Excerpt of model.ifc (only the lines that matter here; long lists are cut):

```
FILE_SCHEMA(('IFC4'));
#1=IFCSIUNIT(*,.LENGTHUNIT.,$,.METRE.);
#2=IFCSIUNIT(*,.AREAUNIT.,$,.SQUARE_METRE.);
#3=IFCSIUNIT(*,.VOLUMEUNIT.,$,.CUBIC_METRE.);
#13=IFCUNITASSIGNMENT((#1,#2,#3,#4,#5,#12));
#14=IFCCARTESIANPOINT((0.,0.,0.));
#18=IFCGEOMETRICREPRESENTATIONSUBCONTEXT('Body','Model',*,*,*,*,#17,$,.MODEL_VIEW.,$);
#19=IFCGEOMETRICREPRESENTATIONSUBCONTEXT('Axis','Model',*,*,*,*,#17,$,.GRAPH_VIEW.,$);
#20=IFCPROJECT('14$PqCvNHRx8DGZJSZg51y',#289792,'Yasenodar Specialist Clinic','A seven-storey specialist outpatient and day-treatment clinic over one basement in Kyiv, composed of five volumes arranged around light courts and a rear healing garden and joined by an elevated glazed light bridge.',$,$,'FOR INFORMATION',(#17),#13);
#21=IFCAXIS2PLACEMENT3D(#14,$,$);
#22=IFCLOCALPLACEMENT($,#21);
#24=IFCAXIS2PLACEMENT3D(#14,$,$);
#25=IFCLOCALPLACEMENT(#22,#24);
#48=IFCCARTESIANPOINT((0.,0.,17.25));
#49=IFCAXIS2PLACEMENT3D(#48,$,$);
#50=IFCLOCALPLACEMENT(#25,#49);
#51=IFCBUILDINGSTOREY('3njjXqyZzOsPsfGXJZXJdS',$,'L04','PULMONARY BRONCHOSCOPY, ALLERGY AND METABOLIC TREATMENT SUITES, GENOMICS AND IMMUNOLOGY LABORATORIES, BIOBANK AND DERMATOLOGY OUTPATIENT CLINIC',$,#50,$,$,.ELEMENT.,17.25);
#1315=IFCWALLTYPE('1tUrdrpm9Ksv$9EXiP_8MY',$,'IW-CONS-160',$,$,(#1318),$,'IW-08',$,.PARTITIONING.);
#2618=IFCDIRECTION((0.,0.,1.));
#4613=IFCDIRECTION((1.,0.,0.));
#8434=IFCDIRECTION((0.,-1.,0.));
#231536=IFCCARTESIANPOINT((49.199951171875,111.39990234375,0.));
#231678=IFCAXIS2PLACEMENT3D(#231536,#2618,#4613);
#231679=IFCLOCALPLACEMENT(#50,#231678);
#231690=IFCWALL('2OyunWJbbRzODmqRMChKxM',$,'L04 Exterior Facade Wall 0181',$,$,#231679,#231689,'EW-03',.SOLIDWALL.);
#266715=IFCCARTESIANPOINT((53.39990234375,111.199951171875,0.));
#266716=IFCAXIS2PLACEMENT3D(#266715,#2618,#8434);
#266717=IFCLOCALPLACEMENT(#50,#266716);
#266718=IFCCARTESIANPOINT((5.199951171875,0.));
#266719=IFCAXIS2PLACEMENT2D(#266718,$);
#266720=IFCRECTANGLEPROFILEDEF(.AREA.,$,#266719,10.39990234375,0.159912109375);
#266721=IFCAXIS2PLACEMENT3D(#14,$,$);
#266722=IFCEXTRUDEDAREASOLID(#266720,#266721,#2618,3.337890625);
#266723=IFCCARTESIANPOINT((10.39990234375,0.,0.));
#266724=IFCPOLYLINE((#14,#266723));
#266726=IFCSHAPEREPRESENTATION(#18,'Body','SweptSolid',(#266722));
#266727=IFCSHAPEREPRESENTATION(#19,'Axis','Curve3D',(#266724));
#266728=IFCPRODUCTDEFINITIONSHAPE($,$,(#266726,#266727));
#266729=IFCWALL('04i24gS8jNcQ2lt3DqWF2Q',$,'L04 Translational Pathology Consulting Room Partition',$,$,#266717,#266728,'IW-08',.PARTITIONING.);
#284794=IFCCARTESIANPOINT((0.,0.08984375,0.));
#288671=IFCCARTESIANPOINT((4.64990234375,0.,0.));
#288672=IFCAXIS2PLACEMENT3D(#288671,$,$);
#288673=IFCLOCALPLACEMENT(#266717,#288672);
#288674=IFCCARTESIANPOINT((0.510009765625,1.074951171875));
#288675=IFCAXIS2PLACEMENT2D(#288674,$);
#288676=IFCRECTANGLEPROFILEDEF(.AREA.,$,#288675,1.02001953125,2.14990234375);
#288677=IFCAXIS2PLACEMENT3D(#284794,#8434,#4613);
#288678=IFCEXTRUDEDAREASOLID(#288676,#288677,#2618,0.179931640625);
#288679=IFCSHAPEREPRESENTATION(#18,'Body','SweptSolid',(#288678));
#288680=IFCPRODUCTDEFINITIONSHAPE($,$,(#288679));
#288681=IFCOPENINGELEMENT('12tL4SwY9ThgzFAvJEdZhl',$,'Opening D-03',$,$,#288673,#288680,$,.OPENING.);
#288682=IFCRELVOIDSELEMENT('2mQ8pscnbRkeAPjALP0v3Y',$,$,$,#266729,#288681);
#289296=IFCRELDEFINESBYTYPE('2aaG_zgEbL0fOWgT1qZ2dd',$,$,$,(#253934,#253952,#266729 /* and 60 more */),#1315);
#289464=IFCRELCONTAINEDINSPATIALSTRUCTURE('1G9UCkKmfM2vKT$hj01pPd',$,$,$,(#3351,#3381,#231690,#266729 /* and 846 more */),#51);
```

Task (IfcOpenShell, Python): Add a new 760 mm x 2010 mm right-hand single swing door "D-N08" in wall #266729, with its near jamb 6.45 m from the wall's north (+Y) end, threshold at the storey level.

```python
import numpy as np
import ifcopenshell
import ifcopenshell.api.feature
import ifcopenshell.api.geometry
import ifcopenshell.api.root
import ifcopenshell.api.spatial
import ifcopenshell.geom
import ifcopenshell.util.element
import ifcopenshell.util.placement
import ifcopenshell.util.representation
import ifcopenshell.util.shape
import ifcopenshell.util.unit

model = ifcopenshell.open("model.ifc")
unit_scale = ifcopenshell.util.unit.calculate_unit_scale(model)
settings = ifcopenshell.geom.settings()


def volume(element):
    """Net volume in cubic metres, openings subtracted."""
    shape = ifcopenshell.geom.create_shape(settings, element)
    return ifcopenshell.util.shape.get_volume(shape.geometry)


wall = model.by_id(266729)
storey = ifcopenshell.util.element.get_container(wall, ifc_class="IfcBuildingStorey")
context = ifcopenshell.util.representation.get_context(model, "Model", "Body", "MODEL_VIEW")
before = volume(wall)

width, height, from_end, sill = 0.76, 2.01, 6.45, 0.0  # metres

# The wall runs along its own X axis, and the end named is its -X end.
wall_shape = ifcopenshell.geom.create_shape(settings, wall)
x, y, z = ifcopenshell.util.shape.get_vertices(wall_shape.geometry).T
start = x.min() + from_end
face, thickness = float(y.min()), float(y.max() - y.min())
wall_matrix = ifcopenshell.util.placement.get_local_placement(wall.ObjectPlacement)
level = ifcopenshell.util.placement.get_local_placement(storey.ObjectPlacement)[2, 3]


def in_wall(x, y):
    """Placement at x, y metres in the wall's axes, at sill height."""
    matrix = wall_matrix.copy()
    matrix[:, 3] = wall_matrix @ np.array([x / unit_scale, y / unit_scale, 0.0, 1.0])
    matrix[2, 3] = level + sill / unit_scale
    return matrix


# Opening: a box that overshoots both wall faces by 50 mm.
opening = ifcopenshell.api.root.create_entity(model, ifc_class="IfcOpeningElement", predefined_type="OPENING")
box = ifcopenshell.api.geometry.add_wall_representation(
    model, context=context, length=width, height=height, thickness=thickness + 0.1
)
ifcopenshell.api.geometry.assign_representation(model, product=opening, representation=box)
ifcopenshell.api.geometry.edit_object_placement(model, product=opening, matrix=in_wall(start, face - 0.05), is_si=False)
ifcopenshell.api.feature.add_feature(model, feature=opening, element=wall)

door = ifcopenshell.api.root.create_entity(model, ifc_class="IfcDoor", name="D-N08", predefined_type="DOOR")
door.OverallWidth, door.OverallHeight = width / unit_scale, height / unit_scale
door.OperationType = "SINGLE_SWING_RIGHT"
body = ifcopenshell.api.geometry.add_door_representation(
    model,
    context=context,
    overall_width=door.OverallWidth,
    overall_height=door.OverallHeight,
    operation_type="SINGLE_SWING_RIGHT",
    lining_properties={"LiningDepth": thickness / unit_scale, "ThresholdDepth": thickness / unit_scale},
)
ifcopenshell.api.geometry.assign_representation(model, product=door, representation=body)
ifcopenshell.api.spatial.assign_container(model, products=[door], relating_structure=storey)
ifcopenshell.api.feature.add_filling(model, opening=opening, element=door)

# The lining spans the wall, so the door starts at the wall face.
ifcopenshell.api.geometry.edit_object_placement(model, product=door, matrix=in_wall(start, face), is_si=False)

after = volume(wall)

print(f"wall volume {before:.3f} -> {after:.3f} m3")

model.write("model_edited.ifc")
```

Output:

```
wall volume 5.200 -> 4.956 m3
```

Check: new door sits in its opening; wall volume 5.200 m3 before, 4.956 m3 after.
